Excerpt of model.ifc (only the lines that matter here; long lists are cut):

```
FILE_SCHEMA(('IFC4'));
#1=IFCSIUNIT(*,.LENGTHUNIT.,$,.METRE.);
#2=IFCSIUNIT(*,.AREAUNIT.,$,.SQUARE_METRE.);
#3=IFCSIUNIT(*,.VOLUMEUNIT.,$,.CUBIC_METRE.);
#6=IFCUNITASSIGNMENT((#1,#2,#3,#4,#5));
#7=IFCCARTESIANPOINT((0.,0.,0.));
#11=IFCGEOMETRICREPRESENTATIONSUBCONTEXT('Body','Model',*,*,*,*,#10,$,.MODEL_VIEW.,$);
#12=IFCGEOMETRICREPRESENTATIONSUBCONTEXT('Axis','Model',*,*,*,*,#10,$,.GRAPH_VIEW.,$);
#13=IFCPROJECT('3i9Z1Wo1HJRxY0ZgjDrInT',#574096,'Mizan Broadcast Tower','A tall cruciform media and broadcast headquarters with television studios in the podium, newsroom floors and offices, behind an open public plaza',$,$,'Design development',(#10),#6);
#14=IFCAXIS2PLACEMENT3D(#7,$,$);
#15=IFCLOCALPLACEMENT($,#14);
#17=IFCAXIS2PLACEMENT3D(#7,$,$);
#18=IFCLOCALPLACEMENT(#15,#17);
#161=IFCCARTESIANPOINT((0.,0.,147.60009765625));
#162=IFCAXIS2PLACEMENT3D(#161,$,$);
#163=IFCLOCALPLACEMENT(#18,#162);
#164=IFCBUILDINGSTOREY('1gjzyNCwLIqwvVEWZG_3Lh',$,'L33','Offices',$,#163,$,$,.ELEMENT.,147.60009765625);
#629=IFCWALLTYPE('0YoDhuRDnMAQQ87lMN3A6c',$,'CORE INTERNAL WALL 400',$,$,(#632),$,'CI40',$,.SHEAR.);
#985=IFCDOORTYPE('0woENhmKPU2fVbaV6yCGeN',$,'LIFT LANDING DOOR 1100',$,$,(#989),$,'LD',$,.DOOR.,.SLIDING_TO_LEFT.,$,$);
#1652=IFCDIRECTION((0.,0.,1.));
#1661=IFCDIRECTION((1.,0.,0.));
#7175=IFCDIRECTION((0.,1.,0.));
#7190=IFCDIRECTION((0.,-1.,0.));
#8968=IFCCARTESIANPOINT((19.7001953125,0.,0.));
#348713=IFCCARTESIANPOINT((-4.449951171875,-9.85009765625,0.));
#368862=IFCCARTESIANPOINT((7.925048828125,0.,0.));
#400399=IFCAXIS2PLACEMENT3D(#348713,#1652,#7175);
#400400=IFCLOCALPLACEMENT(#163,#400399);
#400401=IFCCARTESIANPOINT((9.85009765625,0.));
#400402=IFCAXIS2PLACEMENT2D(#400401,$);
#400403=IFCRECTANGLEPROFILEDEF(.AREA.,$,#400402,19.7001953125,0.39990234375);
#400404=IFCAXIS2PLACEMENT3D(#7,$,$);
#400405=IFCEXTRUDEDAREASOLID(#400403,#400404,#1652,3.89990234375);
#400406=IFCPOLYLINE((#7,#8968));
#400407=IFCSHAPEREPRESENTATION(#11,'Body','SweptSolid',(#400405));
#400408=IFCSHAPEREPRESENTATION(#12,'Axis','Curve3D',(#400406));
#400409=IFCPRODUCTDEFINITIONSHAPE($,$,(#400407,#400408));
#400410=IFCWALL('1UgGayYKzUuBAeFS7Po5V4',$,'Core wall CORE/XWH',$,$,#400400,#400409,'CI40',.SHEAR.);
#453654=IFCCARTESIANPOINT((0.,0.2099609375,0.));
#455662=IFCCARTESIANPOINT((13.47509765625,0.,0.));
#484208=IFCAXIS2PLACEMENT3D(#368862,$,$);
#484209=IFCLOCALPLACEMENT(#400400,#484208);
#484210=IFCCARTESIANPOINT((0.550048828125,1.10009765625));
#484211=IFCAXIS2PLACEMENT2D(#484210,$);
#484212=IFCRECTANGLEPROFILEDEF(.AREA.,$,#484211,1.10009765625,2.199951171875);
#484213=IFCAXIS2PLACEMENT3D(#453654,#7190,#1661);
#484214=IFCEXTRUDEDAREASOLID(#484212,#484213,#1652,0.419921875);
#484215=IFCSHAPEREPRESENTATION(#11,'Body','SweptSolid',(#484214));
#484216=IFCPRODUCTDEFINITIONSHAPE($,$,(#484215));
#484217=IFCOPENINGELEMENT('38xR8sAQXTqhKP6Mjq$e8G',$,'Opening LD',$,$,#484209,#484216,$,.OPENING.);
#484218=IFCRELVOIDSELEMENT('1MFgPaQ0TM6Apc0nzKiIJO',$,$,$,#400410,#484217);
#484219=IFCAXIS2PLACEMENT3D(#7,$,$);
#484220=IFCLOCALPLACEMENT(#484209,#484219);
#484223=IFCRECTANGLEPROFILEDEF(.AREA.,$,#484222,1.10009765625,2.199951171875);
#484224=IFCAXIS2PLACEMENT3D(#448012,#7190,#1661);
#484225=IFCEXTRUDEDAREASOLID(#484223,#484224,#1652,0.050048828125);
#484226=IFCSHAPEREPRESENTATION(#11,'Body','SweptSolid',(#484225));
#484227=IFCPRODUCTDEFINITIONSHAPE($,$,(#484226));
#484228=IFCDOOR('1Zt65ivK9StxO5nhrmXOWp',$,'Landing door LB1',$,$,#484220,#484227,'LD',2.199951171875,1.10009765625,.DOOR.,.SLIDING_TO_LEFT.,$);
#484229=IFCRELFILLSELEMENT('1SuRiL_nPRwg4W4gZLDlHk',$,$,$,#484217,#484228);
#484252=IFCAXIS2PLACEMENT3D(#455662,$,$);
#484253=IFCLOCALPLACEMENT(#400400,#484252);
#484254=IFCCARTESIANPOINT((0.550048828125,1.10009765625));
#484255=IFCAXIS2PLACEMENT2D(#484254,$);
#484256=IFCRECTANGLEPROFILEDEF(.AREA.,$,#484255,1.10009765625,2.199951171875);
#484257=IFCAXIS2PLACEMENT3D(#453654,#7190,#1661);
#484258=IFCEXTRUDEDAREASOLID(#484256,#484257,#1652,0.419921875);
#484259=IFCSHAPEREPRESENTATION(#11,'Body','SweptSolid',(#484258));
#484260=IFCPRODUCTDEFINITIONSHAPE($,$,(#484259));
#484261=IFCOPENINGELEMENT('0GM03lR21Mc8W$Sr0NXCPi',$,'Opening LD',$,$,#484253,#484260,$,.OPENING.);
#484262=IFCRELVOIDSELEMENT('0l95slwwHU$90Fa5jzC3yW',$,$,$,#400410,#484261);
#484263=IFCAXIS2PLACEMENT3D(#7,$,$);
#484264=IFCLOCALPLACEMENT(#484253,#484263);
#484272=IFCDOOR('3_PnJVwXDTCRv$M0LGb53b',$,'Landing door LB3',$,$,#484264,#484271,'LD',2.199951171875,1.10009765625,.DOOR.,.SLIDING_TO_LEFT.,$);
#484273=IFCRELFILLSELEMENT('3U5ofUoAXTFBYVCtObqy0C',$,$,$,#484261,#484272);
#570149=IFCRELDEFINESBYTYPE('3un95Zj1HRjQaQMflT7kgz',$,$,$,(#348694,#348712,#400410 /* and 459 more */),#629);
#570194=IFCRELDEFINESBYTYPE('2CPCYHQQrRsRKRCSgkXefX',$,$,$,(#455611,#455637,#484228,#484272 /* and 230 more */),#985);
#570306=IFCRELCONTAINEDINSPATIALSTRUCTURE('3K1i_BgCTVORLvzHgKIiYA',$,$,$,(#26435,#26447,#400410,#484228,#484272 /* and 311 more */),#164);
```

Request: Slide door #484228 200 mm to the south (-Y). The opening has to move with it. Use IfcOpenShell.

```python
import ifcopenshell
import ifcopenshell.api.geometry
import ifcopenshell.util.placement
import ifcopenshell.util.unit

model = ifcopenshell.open("model.ifc")
unit_scale = ifcopenshell.util.unit.calculate_unit_scale(model)

door = model.by_guid("1Zt65ivK9StxO5nhrmXOWp")
opening = door.FillsVoids[0].RelatingOpeningElement
wall = opening.VoidsElements[0].RelatingBuildingElement

wall_matrix = ifcopenshell.util.placement.get_local_placement(wall.ObjectPlacement)
shift = wall_matrix[:3, 0] * -0.2 / unit_scale
before = ifcopenshell.util.placement.get_local_placement(door.ObjectPlacement)[:3, 3].copy()

# The door is placed relative to its opening, so it follows when the opening moves.
matrix = ifcopenshell.util.placement.get_local_placement(opening.ObjectPlacement)
matrix[:3, 3] += shift
ifcopenshell.api.geometry.edit_object_placement(
    model, product=opening, matrix=matrix, is_si=False, should_transform_children=True
)

after = ifcopenshell.util.placement.get_local_placement(door.ObjectPlacement)[:3, 3]
print("door moved by", (after - before).round(3) + 0.0)

model.write("model-out.ifc")
```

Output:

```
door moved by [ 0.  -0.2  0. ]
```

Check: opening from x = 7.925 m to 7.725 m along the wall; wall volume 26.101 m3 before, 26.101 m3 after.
